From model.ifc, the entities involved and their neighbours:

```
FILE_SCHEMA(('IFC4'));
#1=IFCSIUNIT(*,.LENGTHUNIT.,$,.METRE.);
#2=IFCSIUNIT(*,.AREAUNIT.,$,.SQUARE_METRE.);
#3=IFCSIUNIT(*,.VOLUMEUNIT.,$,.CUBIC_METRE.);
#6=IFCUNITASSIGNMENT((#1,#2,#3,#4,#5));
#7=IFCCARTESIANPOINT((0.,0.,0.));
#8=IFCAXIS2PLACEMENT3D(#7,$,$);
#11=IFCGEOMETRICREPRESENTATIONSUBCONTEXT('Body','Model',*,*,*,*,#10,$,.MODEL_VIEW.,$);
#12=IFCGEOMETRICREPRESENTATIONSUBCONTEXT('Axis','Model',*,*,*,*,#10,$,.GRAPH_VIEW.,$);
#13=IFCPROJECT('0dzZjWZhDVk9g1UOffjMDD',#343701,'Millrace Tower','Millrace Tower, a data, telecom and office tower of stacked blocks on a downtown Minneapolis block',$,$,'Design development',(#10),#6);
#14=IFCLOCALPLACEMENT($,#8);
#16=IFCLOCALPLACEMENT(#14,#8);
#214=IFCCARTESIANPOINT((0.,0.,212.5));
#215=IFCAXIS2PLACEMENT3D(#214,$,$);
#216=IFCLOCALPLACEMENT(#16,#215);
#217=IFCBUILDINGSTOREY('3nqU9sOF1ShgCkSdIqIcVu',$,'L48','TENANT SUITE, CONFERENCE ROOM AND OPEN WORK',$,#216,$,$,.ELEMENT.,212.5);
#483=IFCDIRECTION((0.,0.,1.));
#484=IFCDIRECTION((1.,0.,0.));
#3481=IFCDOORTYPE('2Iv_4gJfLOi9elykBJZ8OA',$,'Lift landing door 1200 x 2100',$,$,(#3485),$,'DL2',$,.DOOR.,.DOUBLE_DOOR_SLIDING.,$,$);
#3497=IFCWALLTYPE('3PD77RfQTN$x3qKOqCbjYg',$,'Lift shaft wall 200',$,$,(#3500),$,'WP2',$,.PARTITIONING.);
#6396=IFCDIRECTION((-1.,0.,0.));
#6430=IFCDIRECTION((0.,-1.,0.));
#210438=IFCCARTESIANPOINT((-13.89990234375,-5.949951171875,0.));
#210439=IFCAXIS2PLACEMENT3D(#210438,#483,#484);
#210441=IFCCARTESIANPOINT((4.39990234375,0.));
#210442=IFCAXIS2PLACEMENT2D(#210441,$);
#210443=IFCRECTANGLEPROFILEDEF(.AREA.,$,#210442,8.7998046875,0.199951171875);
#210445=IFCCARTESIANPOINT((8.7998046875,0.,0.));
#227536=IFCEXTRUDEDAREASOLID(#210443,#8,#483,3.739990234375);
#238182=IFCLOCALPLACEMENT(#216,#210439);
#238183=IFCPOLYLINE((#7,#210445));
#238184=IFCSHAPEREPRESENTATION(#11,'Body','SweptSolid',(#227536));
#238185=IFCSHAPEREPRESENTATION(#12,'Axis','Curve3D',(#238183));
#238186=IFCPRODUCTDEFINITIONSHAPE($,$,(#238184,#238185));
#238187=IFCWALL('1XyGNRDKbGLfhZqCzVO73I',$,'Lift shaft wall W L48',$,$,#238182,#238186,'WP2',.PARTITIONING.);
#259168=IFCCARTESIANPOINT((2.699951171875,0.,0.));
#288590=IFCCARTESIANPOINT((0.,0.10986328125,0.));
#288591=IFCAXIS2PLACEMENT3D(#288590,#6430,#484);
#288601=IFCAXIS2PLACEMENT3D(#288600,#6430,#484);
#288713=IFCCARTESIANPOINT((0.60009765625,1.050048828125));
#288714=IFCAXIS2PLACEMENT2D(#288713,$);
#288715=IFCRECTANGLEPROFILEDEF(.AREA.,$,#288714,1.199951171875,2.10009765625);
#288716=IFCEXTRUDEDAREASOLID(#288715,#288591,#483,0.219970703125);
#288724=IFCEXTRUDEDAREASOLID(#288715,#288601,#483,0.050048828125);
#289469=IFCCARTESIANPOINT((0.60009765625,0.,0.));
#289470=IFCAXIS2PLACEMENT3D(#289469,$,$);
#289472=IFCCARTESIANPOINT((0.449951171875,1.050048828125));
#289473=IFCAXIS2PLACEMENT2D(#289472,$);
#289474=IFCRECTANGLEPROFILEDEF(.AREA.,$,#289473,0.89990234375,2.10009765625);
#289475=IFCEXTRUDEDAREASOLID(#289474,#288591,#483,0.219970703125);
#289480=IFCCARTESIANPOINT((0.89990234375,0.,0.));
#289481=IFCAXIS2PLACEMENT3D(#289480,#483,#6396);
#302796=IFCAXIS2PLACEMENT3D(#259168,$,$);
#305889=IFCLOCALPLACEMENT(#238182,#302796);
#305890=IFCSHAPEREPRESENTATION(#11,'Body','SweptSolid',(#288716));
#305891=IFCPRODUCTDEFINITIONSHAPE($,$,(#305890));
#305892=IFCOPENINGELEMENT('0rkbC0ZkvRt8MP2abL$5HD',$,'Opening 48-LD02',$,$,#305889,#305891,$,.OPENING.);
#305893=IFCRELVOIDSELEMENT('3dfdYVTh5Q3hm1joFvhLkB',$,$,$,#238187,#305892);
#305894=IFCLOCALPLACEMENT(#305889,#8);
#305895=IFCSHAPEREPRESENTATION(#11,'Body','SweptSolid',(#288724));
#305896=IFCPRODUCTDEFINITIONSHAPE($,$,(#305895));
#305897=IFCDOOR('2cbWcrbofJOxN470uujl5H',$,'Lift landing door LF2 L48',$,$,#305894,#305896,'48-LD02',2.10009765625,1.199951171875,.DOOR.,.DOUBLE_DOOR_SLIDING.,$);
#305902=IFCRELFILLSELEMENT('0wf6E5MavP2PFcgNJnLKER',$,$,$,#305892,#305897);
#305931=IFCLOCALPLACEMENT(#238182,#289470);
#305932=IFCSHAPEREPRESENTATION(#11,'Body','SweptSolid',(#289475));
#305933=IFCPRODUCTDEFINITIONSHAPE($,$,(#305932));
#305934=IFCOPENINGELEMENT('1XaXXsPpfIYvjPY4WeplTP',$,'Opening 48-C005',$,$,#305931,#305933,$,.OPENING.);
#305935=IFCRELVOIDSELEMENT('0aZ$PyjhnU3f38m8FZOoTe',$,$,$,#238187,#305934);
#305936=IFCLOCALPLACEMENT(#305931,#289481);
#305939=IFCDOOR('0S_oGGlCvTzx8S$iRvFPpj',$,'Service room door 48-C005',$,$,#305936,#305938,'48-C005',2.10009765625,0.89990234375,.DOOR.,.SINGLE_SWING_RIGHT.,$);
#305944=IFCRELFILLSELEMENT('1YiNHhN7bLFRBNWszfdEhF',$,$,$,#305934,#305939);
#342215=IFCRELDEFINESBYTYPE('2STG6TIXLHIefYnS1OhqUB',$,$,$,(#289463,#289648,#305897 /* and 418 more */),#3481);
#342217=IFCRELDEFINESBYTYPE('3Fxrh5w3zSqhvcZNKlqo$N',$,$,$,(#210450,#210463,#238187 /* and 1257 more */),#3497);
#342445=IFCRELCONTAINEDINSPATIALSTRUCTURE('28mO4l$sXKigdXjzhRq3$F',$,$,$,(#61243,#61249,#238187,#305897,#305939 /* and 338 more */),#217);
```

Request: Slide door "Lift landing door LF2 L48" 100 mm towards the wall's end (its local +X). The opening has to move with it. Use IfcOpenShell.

```python
import ifcopenshell
import ifcopenshell.api.geometry
import ifcopenshell.util.placement
import ifcopenshell.util.unit

model = ifcopenshell.open("model.ifc")
unit_scale = ifcopenshell.util.unit.calculate_unit_scale(model)

door = model.by_id(305897)
opening = door.FillsVoids[0].RelatingOpeningElement
wall = opening.VoidsElements[0].RelatingBuildingElement

wall_matrix = ifcopenshell.util.placement.get_local_placement(wall.ObjectPlacement)
shift = wall_matrix[:3, 0] * 0.1 / unit_scale
before = ifcopenshell.util.placement.get_local_placement(door.ObjectPlacement)[:3, 3].copy()

# The door is placed relative to its opening, so it follows when the opening moves.
matrix = ifcopenshell.util.placement.get_local_placement(opening.ObjectPlacement)
matrix[:3, 3] += shift
ifcopenshell.api.geometry.edit_object_placement(
    model, product=opening, matrix=matrix, is_si=False, should_transform_children=True
)

after = ifcopenshell.util.placement.get_local_placement(door.ObjectPlacement)[:3, 3]
print("door moved by", (after - before).round(3) + 0.0)

model.write("model_updated.ifc")
```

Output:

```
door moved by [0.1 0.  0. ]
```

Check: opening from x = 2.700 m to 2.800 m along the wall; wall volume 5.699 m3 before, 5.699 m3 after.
